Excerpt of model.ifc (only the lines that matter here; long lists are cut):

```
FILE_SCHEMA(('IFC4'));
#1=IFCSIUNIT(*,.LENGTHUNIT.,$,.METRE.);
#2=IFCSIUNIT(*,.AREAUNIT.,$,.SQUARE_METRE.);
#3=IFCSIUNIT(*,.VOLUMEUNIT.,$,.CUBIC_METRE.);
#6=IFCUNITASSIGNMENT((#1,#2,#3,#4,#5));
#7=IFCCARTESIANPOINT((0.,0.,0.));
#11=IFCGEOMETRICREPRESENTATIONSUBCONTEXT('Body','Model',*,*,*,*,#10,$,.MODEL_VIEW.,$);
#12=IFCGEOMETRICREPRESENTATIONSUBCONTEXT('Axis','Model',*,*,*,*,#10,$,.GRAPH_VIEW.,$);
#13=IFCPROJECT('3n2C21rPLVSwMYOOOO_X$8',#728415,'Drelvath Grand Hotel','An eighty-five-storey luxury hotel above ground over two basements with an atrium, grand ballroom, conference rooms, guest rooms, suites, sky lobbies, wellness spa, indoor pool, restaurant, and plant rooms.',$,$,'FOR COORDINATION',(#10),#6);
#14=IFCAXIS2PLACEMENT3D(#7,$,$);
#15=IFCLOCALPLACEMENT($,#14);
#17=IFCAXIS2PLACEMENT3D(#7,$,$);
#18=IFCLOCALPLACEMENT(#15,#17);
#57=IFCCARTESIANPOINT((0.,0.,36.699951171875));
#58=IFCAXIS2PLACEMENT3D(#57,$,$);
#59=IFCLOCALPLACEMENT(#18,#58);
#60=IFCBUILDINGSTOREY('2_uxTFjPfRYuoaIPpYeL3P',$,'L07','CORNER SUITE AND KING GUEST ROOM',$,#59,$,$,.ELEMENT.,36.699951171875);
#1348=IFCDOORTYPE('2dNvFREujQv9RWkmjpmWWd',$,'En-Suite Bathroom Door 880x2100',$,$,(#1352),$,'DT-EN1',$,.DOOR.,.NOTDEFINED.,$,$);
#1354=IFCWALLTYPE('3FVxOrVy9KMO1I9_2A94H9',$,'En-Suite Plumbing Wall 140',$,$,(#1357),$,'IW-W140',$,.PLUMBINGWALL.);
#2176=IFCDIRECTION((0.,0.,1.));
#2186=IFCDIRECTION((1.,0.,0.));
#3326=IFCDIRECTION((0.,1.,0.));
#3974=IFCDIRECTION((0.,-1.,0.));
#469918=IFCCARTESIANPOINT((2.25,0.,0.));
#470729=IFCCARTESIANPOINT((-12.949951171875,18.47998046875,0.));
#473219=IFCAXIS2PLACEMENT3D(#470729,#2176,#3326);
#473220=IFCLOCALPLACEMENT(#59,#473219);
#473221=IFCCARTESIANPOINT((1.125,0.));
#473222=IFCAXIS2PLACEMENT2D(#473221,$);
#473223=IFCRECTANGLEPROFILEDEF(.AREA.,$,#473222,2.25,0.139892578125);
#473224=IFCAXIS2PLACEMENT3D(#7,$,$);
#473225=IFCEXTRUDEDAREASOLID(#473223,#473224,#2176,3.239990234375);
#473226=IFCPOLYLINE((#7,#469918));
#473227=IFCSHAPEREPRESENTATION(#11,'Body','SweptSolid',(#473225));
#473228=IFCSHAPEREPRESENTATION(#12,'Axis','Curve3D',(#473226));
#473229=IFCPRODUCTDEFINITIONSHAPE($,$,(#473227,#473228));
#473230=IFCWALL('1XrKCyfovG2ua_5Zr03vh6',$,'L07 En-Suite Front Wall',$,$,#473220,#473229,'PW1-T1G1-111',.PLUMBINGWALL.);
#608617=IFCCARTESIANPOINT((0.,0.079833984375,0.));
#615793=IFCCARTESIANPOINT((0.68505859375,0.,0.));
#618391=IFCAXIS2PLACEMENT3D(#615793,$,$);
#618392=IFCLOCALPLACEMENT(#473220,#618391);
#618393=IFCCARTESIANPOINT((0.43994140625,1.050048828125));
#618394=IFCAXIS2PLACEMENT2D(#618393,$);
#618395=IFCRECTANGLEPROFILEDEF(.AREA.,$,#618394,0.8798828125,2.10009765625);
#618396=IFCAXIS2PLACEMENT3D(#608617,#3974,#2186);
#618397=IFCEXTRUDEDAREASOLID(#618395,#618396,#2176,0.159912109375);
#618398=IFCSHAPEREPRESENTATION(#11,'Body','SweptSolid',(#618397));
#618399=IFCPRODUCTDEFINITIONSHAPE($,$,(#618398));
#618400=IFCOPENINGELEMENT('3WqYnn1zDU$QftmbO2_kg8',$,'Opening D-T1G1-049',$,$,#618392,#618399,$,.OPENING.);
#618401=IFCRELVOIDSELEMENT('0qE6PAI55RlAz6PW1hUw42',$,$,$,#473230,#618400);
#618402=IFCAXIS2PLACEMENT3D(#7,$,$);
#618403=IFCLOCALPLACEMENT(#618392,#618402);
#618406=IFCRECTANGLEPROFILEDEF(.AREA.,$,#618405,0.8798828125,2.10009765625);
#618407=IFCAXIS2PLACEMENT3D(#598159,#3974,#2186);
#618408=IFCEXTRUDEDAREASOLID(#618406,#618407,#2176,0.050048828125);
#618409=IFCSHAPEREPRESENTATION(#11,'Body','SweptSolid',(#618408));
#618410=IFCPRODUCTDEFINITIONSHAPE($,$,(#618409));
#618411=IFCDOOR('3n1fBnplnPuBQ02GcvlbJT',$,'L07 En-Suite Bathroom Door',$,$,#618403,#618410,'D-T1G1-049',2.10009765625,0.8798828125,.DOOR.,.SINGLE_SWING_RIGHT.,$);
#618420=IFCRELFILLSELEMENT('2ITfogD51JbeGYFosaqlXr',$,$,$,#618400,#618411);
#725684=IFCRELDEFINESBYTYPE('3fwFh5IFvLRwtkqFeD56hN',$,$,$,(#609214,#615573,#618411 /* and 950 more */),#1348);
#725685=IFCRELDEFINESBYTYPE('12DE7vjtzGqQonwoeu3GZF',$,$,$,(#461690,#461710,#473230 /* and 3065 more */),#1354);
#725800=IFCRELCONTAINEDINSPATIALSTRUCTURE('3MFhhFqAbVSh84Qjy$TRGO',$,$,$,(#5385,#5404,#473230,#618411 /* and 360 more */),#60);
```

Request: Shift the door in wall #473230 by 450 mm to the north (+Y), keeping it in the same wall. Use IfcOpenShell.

```python
import ifcopenshell
import ifcopenshell.api.geometry
import ifcopenshell.util.placement

model = ifcopenshell.open("model.ifc")

door = model.by_guid("3n1fBnplnPuBQ02GcvlbJT")
opening = door.FillsVoids[0].RelatingOpeningElement
wall = opening.VoidsElements[0].RelatingBuildingElement

wall_matrix = ifcopenshell.util.placement.get_local_placement(wall.ObjectPlacement)
shift = wall_matrix[:3, 0] * 0.45
before = ifcopenshell.util.placement.get_local_placement(door.ObjectPlacement)[:3, 3].copy()

# The door is placed relative to its opening, so it follows when the opening moves.
matrix = ifcopenshell.util.placement.get_local_placement(opening.ObjectPlacement)
matrix[:3, 3] += shift
ifcopenshell.api.geometry.edit_object_placement(
    model, product=opening, matrix=matrix, is_si=False, should_transform_children=True
)

after = ifcopenshell.util.placement.get_local_placement(door.ObjectPlacement)[:3, 3]
print("door moved by", (after - before).round(3) + 0.0)

model.write("model_v2.ifc")
```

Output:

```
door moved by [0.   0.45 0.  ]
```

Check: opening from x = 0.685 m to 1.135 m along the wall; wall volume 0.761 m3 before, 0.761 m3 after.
